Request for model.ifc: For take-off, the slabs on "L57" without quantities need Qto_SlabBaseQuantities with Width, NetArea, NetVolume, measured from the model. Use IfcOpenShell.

First a look at what the model holds.

```python
import ifcopenshell
import ifcopenshell.util.element
import ifcopenshell.util.unit

model = ifcopenshell.open("model.ifc")
print(model.schema)
for unit_type in ("LENGTHUNIT", "AREAUNIT", "VOLUMEUNIT"):
    print(unit_type, ifcopenshell.util.unit.calculate_unit_scale(model, unit_type))
storey = next(s for s in model.by_type("IfcBuildingStorey") if s.Name == "L57")
slabs = [e for e in ifcopenshell.util.element.get_decomposition(storey) if e.is_a("IfcSlab")]
for e in sorted(slabs, key=lambda e: e.id()):
    print(e.id(), e.is_a(), e.Name, list(ifcopenshell.util.element.get_psets(e, qtos_only=True)), sep=" | ")
```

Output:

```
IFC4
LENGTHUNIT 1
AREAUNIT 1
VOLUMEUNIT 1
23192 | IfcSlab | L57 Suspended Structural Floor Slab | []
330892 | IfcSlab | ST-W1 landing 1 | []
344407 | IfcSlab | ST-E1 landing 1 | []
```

```python
import ifcopenshell
import ifcopenshell.api.pset
import ifcopenshell.geom
import ifcopenshell.util.element
import ifcopenshell.util.shape
import ifcopenshell.util.unit

model = ifcopenshell.open("model.ifc")
unit_scale = ifcopenshell.util.unit.calculate_unit_scale(model)
area_scale = ifcopenshell.util.unit.calculate_unit_scale(model, "AREAUNIT")
volume_scale = ifcopenshell.util.unit.calculate_unit_scale(model, "VOLUMEUNIT")
settings = ifcopenshell.geom.settings()

storey = next(s for s in model.by_type("IfcBuildingStorey") if s.Name == "L57")
slabs = [e for e in ifcopenshell.util.element.get_decomposition(storey) if e.is_a("IfcSlab")]

for e in sorted(slabs, key=lambda e: e.id()):
    if ifcopenshell.util.element.get_psets(e, qtos_only=True, should_inherit=False):
        continue
    # Geometry comes back in metres, in the element's own axes.
    shape = ifcopenshell.geom.create_shape(settings, e)
    values = {
        "Width": ifcopenshell.util.shape.get_z(shape.geometry) / unit_scale,
        "NetArea": ifcopenshell.util.shape.get_footprint_area(shape.geometry) / area_scale,
        "NetVolume": ifcopenshell.util.shape.get_volume(shape.geometry) / volume_scale,
    }
    qto = ifcopenshell.api.pset.add_qto(model, product=e, name="Qto_SlabBaseQuantities")
    ifcopenshell.api.pset.edit_qto(model, qto=qto, properties=values)
    print(e.id(), {k: round(v, 3) for k, v in values.items()})

model.write("model_rev.ifc")
```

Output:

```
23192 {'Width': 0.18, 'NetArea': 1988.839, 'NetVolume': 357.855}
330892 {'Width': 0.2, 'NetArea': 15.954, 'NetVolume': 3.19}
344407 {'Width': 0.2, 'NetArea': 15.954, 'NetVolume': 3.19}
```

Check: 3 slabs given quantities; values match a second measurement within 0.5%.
